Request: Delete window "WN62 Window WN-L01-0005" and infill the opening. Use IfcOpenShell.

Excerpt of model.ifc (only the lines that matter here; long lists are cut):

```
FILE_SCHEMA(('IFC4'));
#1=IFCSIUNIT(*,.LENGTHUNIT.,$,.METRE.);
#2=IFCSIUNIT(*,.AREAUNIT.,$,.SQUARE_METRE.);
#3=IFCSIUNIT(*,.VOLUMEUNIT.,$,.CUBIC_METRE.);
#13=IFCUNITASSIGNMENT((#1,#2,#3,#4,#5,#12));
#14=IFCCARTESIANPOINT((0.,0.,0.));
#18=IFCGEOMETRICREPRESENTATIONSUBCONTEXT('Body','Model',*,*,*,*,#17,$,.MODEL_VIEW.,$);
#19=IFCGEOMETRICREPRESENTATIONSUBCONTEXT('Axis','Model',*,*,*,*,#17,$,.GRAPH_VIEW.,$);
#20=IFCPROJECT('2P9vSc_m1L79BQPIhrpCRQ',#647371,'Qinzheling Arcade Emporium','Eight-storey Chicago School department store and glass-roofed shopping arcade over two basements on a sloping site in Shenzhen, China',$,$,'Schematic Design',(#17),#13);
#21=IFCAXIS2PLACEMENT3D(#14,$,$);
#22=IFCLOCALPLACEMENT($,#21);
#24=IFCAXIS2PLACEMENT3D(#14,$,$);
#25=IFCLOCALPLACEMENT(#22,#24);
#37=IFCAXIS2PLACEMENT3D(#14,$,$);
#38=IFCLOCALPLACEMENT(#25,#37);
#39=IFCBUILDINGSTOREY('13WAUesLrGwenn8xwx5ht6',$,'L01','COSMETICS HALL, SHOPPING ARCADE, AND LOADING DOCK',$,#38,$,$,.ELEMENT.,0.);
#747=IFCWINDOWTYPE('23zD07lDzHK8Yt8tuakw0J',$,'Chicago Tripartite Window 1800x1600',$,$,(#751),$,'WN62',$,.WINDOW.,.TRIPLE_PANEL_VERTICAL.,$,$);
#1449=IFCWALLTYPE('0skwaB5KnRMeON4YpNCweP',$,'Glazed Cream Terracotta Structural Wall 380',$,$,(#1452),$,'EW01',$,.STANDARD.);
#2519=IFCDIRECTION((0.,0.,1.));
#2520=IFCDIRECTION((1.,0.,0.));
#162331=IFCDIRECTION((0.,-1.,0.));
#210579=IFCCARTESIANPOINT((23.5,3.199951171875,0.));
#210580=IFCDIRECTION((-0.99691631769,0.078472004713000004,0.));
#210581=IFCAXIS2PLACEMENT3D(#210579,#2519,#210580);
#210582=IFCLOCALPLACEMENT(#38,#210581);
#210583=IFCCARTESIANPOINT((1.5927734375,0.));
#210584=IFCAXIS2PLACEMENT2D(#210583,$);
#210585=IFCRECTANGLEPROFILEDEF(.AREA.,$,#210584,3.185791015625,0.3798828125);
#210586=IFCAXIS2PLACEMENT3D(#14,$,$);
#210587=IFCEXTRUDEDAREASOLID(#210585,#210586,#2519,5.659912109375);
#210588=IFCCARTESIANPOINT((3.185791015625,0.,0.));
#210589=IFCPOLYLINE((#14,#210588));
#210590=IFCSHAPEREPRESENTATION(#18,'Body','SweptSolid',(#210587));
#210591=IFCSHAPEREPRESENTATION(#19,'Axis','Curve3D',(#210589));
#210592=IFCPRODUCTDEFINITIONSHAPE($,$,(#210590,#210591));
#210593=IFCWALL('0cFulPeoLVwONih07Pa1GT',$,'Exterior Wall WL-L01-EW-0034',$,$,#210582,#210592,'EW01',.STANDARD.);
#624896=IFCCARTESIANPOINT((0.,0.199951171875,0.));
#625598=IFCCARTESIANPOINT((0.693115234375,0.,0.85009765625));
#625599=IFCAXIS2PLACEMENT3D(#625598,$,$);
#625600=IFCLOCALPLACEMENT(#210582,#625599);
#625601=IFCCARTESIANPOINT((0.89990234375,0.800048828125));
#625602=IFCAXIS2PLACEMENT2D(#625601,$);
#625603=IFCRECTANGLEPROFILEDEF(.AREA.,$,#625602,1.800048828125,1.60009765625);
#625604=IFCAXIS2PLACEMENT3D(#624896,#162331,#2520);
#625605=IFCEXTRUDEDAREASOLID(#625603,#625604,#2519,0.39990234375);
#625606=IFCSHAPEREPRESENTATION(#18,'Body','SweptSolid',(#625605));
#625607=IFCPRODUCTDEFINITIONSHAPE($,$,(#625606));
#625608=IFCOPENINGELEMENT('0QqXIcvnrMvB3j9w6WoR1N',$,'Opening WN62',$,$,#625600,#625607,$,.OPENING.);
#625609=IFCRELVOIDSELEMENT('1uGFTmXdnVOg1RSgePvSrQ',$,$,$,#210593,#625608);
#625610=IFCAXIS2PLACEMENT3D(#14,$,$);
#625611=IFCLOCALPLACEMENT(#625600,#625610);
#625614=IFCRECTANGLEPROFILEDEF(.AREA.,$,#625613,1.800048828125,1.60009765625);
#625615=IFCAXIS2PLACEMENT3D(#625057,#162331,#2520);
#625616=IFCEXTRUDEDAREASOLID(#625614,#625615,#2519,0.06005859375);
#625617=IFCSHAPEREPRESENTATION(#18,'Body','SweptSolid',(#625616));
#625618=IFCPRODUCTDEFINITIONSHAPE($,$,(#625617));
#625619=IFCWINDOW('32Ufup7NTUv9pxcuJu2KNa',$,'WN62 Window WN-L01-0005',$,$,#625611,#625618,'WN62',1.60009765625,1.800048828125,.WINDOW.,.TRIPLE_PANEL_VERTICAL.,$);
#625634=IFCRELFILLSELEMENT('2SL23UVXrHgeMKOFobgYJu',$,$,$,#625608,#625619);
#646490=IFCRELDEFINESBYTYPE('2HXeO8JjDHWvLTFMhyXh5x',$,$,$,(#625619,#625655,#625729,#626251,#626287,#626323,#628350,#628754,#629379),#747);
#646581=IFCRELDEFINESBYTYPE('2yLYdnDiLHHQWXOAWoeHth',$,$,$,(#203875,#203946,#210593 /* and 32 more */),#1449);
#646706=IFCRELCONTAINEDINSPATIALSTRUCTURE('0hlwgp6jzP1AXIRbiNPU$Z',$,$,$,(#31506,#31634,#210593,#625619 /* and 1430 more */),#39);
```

```python
import ifcopenshell
import ifcopenshell.api.feature
import ifcopenshell.api.root
import ifcopenshell.geom
import ifcopenshell.util.shape

model = ifcopenshell.open("model.ifc")
settings = ifcopenshell.geom.settings()


def volume(element):
    """Net volume in cubic metres, openings subtracted."""
    shape = ifcopenshell.geom.create_shape(settings, element)
    return ifcopenshell.util.shape.get_volume(shape.geometry)


window = model.by_guid("32Ufup7NTUv9pxcuJu2KNa")
opening = window.FillsVoids[0].RelatingOpeningElement
wall = opening.VoidsElements[0].RelatingBuildingElement
before = volume(wall)

ifcopenshell.api.root.remove_product(model, product=window)
ifcopenshell.api.feature.remove_feature(model, feature=opening)

after = volume(wall)

print(f"wall volume {before:.3f} -> {after:.3f} m3")

model.write("model_rev.ifc")
```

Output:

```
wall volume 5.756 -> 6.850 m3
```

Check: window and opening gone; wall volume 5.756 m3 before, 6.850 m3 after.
